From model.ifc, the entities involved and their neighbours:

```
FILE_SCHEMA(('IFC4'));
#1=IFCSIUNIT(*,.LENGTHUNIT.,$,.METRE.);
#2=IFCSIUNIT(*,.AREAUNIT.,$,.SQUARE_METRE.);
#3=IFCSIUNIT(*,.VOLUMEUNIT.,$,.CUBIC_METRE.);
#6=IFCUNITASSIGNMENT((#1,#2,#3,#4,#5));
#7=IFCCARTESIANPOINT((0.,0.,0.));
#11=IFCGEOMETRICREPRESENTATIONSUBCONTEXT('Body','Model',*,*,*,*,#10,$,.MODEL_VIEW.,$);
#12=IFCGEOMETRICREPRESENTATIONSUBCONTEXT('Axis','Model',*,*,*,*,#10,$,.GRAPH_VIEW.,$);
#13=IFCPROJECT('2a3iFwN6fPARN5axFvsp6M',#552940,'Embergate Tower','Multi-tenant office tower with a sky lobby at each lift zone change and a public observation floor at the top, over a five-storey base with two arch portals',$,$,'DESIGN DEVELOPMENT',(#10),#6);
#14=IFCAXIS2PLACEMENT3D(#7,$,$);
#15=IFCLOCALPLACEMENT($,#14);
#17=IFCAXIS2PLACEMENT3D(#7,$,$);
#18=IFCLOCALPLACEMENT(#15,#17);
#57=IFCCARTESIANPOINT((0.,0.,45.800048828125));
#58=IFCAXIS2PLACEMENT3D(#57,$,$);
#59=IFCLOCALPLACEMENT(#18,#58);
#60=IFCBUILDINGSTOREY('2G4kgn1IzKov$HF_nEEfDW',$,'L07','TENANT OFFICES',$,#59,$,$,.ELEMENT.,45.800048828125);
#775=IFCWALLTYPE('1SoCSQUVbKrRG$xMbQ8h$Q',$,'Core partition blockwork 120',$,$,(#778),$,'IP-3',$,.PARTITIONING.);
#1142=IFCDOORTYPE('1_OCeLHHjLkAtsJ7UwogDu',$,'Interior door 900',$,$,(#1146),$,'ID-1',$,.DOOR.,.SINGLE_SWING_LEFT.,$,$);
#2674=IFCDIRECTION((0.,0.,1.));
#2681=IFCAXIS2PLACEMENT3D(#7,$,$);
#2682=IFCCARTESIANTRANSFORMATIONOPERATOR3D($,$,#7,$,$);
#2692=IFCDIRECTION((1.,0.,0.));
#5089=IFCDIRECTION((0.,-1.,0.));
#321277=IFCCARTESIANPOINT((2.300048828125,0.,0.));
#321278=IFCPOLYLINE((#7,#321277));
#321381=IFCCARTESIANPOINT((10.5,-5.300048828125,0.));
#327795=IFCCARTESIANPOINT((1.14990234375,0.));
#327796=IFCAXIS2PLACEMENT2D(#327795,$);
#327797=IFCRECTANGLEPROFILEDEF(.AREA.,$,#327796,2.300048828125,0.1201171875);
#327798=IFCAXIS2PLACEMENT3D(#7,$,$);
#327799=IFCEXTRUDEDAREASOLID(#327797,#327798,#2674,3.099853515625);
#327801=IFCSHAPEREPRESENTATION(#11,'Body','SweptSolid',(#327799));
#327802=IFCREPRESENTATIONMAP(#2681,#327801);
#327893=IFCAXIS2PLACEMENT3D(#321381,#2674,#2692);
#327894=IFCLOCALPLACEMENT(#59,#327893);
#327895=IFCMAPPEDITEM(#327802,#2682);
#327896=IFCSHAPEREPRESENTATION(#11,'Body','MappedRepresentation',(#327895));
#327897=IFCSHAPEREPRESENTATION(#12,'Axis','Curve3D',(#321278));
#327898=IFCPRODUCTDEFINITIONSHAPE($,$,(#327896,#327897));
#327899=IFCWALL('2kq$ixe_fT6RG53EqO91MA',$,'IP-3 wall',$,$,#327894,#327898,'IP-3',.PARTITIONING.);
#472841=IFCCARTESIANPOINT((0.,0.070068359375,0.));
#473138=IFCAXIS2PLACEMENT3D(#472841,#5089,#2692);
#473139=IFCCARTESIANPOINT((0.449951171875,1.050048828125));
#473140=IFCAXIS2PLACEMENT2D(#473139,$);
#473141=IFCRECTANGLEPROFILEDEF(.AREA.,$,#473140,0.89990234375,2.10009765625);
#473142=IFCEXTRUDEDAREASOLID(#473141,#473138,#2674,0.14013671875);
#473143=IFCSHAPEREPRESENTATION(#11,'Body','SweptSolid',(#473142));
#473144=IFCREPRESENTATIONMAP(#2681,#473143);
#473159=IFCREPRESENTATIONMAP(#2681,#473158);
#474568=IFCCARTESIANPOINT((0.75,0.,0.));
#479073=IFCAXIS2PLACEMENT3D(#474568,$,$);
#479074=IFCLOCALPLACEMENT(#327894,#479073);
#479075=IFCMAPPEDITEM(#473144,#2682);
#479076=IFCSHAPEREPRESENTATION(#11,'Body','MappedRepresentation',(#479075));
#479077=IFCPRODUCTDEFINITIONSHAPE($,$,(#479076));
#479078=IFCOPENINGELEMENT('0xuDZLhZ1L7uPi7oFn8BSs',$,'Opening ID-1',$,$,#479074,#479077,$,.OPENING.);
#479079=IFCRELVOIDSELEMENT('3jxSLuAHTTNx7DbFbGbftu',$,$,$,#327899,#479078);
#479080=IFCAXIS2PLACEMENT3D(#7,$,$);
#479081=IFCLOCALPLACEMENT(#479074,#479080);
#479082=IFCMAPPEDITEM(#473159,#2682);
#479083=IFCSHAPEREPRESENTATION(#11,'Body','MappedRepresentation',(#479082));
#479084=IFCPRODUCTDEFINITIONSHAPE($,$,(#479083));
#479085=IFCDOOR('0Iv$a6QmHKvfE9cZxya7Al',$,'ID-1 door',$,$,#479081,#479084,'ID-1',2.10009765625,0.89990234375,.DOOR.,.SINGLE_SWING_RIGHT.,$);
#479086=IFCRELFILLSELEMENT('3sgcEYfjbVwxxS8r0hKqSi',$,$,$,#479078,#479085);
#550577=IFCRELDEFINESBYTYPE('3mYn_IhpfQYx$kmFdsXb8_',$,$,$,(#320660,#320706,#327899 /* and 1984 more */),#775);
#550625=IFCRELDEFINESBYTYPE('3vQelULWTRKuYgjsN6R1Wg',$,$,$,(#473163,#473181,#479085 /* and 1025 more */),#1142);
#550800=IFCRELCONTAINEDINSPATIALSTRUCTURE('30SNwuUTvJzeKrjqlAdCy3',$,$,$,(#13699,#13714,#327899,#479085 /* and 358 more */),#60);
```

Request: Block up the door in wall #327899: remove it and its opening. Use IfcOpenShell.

```python
import ifcopenshell
import ifcopenshell.api.feature
import ifcopenshell.api.root
import ifcopenshell.geom
import ifcopenshell.util.shape

model = ifcopenshell.open("model.ifc")
settings = ifcopenshell.geom.settings()


def volume(element):
    """Net volume in cubic metres, openings subtracted."""
    shape = ifcopenshell.geom.create_shape(settings, element)
    return ifcopenshell.util.shape.get_volume(shape.geometry)


door = model.by_guid("0Iv$a6QmHKvfE9cZxya7Al")
opening = door.FillsVoids[0].RelatingOpeningElement
wall = opening.VoidsElements[0].RelatingBuildingElement
before = volume(wall)

ifcopenshell.api.root.remove_product(model, product=door)
ifcopenshell.api.feature.remove_feature(model, feature=opening)

after = volume(wall)

print(f"wall volume {before:.3f} -> {after:.3f} m3")

model.write("model_rev.ifc")
```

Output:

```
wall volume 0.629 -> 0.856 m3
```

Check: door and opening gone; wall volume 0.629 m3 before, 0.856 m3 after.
